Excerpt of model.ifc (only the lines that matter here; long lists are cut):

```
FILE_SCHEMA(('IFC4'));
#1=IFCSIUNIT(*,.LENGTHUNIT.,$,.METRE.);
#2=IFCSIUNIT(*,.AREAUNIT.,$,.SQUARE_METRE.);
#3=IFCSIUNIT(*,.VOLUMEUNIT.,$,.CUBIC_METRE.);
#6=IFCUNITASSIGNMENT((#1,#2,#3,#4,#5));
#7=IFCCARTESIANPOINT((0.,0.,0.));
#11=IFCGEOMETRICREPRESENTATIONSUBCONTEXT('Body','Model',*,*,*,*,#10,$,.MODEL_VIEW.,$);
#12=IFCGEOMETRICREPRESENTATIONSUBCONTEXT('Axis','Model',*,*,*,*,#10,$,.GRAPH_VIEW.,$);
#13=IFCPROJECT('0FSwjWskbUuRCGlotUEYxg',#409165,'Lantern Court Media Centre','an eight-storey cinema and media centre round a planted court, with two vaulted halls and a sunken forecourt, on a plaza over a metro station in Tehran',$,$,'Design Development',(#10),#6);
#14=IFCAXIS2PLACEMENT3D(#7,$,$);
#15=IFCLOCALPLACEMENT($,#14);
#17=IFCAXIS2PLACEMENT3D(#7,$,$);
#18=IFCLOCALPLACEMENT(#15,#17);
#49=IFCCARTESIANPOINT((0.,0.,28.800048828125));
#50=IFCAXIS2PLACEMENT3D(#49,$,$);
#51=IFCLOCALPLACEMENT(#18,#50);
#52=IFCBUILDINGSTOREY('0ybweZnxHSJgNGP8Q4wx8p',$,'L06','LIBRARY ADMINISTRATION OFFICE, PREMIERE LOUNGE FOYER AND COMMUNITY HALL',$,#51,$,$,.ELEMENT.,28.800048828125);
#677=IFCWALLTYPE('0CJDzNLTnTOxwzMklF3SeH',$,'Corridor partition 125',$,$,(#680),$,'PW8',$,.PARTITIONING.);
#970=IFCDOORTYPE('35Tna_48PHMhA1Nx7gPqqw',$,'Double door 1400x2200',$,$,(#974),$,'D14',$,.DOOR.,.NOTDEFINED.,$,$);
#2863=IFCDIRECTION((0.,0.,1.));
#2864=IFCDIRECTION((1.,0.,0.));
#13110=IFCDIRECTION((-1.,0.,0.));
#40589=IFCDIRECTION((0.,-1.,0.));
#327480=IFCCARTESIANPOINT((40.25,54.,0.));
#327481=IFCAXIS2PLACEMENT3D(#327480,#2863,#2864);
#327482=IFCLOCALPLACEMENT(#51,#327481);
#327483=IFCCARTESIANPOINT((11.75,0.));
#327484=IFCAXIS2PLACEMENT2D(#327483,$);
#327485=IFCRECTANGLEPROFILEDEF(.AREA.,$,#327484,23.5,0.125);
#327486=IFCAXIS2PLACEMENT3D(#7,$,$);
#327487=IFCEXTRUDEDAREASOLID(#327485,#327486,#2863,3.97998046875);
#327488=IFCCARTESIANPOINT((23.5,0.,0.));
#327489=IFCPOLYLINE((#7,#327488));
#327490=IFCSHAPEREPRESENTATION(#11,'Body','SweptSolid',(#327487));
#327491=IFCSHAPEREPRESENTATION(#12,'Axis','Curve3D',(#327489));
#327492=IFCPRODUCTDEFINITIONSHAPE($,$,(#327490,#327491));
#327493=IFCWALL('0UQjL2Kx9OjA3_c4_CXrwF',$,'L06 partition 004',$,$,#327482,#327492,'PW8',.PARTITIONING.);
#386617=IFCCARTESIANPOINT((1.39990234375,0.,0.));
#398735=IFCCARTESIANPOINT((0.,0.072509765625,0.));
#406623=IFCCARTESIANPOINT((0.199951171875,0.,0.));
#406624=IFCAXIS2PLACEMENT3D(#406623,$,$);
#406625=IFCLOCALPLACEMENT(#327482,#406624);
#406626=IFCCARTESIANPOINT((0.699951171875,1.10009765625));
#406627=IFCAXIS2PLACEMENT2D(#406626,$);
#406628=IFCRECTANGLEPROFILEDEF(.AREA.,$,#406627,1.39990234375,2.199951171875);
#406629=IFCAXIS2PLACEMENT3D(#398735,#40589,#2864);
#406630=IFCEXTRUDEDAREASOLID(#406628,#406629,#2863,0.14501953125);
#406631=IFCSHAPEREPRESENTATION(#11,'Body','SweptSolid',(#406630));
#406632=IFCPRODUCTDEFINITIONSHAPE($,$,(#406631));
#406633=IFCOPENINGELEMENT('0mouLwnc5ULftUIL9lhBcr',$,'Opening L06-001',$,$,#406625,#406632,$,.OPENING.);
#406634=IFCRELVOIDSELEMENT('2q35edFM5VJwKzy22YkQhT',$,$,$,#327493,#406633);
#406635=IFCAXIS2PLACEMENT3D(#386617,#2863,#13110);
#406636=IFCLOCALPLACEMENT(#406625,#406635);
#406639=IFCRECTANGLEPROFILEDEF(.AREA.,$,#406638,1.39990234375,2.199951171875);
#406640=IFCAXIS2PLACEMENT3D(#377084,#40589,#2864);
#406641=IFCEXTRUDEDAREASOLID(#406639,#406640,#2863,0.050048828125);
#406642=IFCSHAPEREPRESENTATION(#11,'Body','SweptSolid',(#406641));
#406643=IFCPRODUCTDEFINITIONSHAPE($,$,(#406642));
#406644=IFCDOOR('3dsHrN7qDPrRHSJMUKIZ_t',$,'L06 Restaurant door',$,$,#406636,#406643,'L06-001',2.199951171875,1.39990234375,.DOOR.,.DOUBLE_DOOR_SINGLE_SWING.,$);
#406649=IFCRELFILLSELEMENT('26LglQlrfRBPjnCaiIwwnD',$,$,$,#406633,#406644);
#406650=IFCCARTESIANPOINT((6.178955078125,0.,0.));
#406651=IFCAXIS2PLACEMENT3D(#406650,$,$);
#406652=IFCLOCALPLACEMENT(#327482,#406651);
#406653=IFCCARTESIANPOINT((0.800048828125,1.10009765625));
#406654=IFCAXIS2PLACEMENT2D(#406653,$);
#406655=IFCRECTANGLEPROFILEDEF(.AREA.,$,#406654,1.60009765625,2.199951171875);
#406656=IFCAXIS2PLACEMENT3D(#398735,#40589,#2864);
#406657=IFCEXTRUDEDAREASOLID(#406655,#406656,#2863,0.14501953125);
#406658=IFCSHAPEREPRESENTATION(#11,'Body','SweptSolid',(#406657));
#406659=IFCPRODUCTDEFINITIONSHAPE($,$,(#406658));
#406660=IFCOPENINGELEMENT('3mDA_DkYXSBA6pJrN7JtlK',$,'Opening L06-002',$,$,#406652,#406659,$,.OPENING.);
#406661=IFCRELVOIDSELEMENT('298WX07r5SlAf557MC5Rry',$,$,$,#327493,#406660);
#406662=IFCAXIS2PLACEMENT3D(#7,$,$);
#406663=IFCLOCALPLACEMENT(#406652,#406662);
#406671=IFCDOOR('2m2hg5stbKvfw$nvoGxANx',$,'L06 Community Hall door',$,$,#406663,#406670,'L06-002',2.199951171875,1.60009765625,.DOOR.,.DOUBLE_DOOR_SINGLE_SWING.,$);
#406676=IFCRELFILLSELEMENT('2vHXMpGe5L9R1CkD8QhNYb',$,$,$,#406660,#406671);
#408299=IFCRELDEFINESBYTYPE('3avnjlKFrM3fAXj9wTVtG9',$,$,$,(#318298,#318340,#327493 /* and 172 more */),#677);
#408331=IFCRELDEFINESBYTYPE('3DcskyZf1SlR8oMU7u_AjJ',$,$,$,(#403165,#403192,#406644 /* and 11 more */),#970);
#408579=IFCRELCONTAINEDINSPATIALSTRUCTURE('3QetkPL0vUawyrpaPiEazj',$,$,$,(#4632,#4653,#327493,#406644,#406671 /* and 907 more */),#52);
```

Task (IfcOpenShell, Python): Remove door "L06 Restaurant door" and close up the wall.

```python
import ifcopenshell
import ifcopenshell.api.feature
import ifcopenshell.api.root
import ifcopenshell.geom
import ifcopenshell.util.shape

model = ifcopenshell.open("model.ifc")
settings = ifcopenshell.geom.settings()


def volume(element):
    """Net volume in cubic metres, openings subtracted."""
    shape = ifcopenshell.geom.create_shape(settings, element)
    return ifcopenshell.util.shape.get_volume(shape.geometry)


door = model.by_id(406644)
opening = door.FillsVoids[0].RelatingOpeningElement
wall = opening.VoidsElements[0].RelatingBuildingElement
before = volume(wall)

ifcopenshell.api.root.remove_product(model, product=door)
ifcopenshell.api.feature.remove_feature(model, feature=opening)

after = volume(wall)

print(f"wall volume {before:.3f} -> {after:.3f} m3")

model.write("model_rev.ifc")
```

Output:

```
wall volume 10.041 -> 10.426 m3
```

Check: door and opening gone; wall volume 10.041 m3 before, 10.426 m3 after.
